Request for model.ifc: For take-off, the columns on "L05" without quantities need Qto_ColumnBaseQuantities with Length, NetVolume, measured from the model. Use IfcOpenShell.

First a look at what the model holds.

```python
import ifcopenshell
import ifcopenshell.util.element
import ifcopenshell.util.unit

model = ifcopenshell.open("model.ifc")
print(model.schema)
for unit_type in ("LENGTHUNIT", "AREAUNIT", "VOLUMEUNIT"):
    print(unit_type, ifcopenshell.util.unit.calculate_unit_scale(model, unit_type))
storey = next(s for s in model.by_type("IfcBuildingStorey") if s.Name == "L05")
columns = [e for e in ifcopenshell.util.element.get_decomposition(storey) if e.is_a("IfcColumn")]
for e in sorted(columns, key=lambda e: e.id()):
    print(e.id(), e.is_a(), e.Name, list(ifcopenshell.util.element.get_psets(e, qtos_only=True)), sep=" | ")
```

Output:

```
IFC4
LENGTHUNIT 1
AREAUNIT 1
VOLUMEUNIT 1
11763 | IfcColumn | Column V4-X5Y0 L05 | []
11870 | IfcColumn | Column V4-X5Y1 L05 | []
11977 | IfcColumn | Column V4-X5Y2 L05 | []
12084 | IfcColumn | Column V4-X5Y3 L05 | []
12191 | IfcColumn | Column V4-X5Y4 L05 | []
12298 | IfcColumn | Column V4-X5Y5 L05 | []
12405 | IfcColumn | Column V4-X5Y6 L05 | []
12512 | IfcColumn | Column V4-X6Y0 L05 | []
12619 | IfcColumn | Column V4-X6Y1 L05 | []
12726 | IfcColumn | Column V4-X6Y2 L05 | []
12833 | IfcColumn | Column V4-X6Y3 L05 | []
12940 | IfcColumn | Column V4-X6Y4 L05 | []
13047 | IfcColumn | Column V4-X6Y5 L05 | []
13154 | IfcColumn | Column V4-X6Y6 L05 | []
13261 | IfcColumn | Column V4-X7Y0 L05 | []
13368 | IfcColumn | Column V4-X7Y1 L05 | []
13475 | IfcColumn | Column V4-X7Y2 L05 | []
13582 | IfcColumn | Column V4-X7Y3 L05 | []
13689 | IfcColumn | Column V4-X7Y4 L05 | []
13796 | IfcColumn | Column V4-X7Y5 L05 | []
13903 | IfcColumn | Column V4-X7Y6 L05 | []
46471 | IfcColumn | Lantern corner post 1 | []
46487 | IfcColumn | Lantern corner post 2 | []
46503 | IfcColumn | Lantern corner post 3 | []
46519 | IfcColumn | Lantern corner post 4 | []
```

```python
import ifcopenshell
import ifcopenshell.api.pset
import ifcopenshell.geom
import ifcopenshell.util.element
import ifcopenshell.util.shape
import ifcopenshell.util.unit

model = ifcopenshell.open("model.ifc")
unit_scale = ifcopenshell.util.unit.calculate_unit_scale(model)
volume_scale = ifcopenshell.util.unit.calculate_unit_scale(model, "VOLUMEUNIT")
settings = ifcopenshell.geom.settings()

storey = next(s for s in model.by_type("IfcBuildingStorey") if s.Name == "L05")
columns = [e for e in ifcopenshell.util.element.get_decomposition(storey) if e.is_a("IfcColumn")]

for e in sorted(columns, key=lambda e: e.id()):
    if ifcopenshell.util.element.get_psets(e, qtos_only=True, should_inherit=False):
        continue
    # Geometry comes back in metres, in the element's own axes.
    shape = ifcopenshell.geom.create_shape(settings, e)
    values = {
        "Length": ifcopenshell.util.shape.get_z(shape.geometry) / unit_scale,
        "NetVolume": ifcopenshell.util.shape.get_volume(shape.geometry) / volume_scale,
    }
    qto = ifcopenshell.api.pset.add_qto(model, product=e, name="Qto_ColumnBaseQuantities")
    ifcopenshell.api.pset.edit_qto(model, qto=qto, properties=values)
    print(e.id(), {k: round(v, 3) for k, v in values.items()})

model.write("model_edited.ifc")
```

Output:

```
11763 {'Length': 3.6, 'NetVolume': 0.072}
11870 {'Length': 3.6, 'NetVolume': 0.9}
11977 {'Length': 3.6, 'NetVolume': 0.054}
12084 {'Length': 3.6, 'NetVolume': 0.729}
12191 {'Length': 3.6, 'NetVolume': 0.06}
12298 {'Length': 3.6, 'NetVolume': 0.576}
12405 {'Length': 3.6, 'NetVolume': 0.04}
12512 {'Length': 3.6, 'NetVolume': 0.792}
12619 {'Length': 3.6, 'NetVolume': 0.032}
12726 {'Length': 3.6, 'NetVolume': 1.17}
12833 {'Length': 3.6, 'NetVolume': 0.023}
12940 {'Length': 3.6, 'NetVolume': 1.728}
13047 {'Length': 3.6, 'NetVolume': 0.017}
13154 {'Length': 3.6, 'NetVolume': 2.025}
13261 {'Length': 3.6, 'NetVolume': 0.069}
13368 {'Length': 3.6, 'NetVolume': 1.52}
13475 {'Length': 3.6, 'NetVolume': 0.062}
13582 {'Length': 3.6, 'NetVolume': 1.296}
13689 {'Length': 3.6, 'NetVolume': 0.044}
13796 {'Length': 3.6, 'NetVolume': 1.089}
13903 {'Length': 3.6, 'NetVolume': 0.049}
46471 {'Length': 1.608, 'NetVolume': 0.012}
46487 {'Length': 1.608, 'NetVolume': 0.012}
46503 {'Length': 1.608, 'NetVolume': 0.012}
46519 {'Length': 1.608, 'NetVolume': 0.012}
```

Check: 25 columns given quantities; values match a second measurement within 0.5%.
